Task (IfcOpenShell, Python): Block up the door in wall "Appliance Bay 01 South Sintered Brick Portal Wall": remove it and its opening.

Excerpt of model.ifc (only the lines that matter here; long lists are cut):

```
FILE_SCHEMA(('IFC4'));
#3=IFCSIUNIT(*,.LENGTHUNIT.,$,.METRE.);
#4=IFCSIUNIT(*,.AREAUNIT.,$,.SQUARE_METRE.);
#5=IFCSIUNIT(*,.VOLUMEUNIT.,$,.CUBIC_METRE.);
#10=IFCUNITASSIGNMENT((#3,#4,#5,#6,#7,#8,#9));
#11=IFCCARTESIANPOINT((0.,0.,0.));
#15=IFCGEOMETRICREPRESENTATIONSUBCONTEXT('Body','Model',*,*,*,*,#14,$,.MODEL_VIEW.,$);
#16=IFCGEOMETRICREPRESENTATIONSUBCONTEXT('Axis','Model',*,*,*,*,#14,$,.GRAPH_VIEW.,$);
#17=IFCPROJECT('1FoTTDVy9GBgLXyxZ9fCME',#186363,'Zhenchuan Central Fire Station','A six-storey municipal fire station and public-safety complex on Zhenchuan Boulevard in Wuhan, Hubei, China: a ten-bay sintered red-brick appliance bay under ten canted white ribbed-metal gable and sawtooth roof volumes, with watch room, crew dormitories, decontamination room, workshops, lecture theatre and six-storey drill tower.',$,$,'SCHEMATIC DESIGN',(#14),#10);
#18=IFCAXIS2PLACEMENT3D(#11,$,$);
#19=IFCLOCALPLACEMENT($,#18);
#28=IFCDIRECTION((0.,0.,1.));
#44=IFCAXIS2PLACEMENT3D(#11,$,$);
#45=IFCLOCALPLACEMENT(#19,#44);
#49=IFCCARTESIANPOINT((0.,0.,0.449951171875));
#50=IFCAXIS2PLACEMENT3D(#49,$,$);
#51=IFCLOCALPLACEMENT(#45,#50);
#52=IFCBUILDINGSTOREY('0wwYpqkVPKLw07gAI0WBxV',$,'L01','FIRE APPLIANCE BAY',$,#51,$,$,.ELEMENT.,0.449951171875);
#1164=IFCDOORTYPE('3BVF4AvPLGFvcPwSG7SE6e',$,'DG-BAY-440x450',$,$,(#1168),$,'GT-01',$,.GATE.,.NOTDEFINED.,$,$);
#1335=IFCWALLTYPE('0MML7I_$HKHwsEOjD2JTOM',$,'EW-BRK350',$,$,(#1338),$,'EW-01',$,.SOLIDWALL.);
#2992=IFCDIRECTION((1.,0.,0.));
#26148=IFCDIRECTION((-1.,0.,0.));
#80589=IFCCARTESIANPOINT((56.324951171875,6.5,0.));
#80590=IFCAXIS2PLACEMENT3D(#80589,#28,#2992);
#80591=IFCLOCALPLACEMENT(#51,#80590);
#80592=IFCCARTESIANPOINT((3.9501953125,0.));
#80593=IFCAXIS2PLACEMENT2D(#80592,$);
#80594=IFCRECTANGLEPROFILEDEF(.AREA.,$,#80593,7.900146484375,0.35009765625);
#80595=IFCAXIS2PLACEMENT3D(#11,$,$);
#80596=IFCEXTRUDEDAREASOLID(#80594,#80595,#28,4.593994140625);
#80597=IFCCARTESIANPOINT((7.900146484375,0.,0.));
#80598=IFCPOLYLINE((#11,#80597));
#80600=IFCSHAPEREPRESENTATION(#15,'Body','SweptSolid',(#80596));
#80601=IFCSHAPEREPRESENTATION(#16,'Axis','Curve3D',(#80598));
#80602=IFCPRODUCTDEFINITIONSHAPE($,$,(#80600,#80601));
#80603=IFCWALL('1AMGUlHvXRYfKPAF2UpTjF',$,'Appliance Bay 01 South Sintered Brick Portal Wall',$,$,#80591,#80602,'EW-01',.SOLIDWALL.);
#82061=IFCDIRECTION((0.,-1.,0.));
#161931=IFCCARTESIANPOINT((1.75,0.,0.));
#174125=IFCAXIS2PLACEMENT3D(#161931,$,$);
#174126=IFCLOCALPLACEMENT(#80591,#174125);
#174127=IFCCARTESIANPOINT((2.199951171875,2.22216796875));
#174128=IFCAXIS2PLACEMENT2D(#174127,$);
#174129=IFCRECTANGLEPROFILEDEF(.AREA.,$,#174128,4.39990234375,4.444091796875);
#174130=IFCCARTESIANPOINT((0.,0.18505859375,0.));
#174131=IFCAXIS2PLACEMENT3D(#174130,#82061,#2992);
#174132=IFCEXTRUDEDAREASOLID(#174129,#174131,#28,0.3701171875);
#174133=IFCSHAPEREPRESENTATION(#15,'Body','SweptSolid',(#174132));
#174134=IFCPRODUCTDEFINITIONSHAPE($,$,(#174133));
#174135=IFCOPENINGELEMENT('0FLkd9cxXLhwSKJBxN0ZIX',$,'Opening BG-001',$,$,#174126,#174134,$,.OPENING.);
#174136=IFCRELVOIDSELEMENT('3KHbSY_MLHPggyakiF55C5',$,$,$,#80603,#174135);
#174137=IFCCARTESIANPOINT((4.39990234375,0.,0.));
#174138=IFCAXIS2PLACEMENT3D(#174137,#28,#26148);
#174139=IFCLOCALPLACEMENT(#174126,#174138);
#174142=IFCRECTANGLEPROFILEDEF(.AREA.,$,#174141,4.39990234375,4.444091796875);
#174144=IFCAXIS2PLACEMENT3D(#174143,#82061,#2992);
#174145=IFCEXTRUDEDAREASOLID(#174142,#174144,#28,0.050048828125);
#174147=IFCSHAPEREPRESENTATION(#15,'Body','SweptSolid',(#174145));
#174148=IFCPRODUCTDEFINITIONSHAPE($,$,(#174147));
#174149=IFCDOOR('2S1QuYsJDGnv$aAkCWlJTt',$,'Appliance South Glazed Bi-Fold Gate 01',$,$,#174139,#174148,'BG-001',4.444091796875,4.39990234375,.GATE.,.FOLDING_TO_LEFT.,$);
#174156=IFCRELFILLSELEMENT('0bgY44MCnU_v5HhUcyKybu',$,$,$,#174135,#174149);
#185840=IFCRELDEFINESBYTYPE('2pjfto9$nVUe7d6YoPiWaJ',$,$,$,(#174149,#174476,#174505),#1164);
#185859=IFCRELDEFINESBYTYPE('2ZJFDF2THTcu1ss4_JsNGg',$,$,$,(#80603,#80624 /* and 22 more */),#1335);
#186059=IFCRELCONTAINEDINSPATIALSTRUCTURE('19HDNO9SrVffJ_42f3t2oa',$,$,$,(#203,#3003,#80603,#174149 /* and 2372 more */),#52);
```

```python
import ifcopenshell
import ifcopenshell.api.feature
import ifcopenshell.api.root
import ifcopenshell.geom
import ifcopenshell.util.shape

model = ifcopenshell.open("model.ifc")
settings = ifcopenshell.geom.settings()


def volume(element):
    """Net volume in cubic metres, openings subtracted."""
    shape = ifcopenshell.geom.create_shape(settings, element)
    return ifcopenshell.util.shape.get_volume(shape.geometry)


door = model.by_id(174149)
opening = door.FillsVoids[0].RelatingOpeningElement
wall = opening.VoidsElements[0].RelatingBuildingElement
before = volume(wall)

ifcopenshell.api.root.remove_product(model, product=door)
ifcopenshell.api.feature.remove_feature(model, feature=opening)

after = volume(wall)

print(f"wall volume {before:.3f} -> {after:.3f} m3")

model.write("model_edited.ifc")
```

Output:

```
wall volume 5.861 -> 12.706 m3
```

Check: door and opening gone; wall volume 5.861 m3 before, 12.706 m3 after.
